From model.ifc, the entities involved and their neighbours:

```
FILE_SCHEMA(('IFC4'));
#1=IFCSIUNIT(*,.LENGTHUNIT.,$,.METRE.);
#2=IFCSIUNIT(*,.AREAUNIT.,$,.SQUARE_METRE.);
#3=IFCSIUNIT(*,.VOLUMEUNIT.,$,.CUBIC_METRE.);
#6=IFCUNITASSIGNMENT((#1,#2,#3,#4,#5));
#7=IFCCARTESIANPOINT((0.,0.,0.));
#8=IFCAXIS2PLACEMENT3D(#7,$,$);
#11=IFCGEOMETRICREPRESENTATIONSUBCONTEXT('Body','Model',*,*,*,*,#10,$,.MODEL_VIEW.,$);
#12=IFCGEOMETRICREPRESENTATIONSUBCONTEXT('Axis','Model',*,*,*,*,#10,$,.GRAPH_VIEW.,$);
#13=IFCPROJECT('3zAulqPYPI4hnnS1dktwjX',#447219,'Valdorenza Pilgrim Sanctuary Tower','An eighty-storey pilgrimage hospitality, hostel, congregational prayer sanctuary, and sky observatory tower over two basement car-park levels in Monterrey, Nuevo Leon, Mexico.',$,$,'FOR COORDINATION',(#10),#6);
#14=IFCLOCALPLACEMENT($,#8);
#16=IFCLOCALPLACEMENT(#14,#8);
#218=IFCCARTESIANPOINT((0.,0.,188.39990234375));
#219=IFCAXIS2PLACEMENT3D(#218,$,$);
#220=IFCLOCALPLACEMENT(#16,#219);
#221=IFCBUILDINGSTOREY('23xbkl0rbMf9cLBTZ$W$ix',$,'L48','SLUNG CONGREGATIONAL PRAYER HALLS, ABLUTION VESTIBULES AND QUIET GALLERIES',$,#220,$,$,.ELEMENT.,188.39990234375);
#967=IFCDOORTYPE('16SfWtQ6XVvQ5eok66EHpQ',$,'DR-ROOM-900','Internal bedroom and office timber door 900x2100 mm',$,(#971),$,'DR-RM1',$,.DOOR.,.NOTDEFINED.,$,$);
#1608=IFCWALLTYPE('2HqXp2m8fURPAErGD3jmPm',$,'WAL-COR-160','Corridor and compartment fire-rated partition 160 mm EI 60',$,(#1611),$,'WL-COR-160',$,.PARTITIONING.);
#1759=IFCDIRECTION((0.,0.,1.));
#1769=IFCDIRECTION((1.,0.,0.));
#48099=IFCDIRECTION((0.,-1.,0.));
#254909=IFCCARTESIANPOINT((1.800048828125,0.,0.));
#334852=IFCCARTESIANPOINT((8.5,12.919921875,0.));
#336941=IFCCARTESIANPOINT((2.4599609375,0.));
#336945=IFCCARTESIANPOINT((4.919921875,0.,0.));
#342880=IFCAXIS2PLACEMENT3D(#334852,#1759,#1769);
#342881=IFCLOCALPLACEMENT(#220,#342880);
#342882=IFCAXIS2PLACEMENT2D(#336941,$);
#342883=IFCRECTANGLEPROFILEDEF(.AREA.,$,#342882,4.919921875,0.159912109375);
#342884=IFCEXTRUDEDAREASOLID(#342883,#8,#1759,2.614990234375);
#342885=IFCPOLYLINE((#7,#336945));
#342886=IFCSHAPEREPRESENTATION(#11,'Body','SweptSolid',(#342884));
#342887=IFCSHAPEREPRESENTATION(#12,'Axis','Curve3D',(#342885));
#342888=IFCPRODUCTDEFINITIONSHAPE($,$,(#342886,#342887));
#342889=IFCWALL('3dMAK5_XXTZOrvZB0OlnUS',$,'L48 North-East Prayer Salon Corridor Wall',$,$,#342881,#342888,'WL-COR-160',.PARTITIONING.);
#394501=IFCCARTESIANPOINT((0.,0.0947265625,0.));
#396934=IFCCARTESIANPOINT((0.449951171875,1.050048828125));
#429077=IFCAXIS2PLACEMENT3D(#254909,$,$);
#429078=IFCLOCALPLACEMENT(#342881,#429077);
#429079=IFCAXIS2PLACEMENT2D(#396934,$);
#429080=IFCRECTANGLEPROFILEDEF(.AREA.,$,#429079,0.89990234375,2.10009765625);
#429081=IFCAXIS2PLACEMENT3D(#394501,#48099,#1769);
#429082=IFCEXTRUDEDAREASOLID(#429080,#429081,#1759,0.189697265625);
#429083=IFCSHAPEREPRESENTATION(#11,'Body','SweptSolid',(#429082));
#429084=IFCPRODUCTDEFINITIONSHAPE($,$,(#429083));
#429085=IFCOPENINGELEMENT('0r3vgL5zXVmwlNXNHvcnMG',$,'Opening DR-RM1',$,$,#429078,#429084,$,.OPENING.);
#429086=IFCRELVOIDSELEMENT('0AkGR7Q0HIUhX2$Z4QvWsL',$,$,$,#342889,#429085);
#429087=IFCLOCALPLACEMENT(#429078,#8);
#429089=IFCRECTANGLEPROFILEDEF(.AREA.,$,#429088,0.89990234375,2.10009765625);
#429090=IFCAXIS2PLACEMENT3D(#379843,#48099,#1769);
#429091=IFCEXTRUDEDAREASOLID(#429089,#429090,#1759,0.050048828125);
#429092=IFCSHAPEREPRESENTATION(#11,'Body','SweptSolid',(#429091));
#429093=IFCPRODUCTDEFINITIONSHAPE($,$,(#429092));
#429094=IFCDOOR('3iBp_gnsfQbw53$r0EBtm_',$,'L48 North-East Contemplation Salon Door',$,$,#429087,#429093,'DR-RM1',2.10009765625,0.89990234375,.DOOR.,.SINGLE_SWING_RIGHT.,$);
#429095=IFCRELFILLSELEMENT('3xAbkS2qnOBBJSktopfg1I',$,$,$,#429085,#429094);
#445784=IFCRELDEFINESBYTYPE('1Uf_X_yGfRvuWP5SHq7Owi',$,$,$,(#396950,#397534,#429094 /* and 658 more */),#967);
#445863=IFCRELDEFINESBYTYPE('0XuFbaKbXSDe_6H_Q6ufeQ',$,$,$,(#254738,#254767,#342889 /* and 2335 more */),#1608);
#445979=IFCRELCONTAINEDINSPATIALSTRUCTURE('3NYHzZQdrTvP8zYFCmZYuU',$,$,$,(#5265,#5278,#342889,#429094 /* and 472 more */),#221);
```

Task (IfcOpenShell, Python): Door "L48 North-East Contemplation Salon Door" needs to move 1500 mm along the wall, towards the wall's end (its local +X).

```python
import ifcopenshell
import ifcopenshell.api.geometry
import ifcopenshell.util.placement
import ifcopenshell.util.unit

model = ifcopenshell.open("model.ifc")
unit_scale = ifcopenshell.util.unit.calculate_unit_scale(model)

door = model.by_guid("3iBp_gnsfQbw53$r0EBtm_")
opening = door.FillsVoids[0].RelatingOpeningElement
wall = opening.VoidsElements[0].RelatingBuildingElement

wall_matrix = ifcopenshell.util.placement.get_local_placement(wall.ObjectPlacement)
shift = wall_matrix[:3, 0] * 1.5 / unit_scale
before = ifcopenshell.util.placement.get_local_placement(door.ObjectPlacement)[:3, 3].copy()

# The door is placed relative to its opening, so it follows when the opening moves.
matrix = ifcopenshell.util.placement.get_local_placement(opening.ObjectPlacement)
matrix[:3, 3] += shift
ifcopenshell.api.geometry.edit_object_placement(
    model, product=opening, matrix=matrix, is_si=False, should_transform_children=True
)

after = ifcopenshell.util.placement.get_local_placement(door.ObjectPlacement)[:3, 3]
print("door moved by", (after - before).round(3) + 0.0)

model.write("model_edited.ifc")
```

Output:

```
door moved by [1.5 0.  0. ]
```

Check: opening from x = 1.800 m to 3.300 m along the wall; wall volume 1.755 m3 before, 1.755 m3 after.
